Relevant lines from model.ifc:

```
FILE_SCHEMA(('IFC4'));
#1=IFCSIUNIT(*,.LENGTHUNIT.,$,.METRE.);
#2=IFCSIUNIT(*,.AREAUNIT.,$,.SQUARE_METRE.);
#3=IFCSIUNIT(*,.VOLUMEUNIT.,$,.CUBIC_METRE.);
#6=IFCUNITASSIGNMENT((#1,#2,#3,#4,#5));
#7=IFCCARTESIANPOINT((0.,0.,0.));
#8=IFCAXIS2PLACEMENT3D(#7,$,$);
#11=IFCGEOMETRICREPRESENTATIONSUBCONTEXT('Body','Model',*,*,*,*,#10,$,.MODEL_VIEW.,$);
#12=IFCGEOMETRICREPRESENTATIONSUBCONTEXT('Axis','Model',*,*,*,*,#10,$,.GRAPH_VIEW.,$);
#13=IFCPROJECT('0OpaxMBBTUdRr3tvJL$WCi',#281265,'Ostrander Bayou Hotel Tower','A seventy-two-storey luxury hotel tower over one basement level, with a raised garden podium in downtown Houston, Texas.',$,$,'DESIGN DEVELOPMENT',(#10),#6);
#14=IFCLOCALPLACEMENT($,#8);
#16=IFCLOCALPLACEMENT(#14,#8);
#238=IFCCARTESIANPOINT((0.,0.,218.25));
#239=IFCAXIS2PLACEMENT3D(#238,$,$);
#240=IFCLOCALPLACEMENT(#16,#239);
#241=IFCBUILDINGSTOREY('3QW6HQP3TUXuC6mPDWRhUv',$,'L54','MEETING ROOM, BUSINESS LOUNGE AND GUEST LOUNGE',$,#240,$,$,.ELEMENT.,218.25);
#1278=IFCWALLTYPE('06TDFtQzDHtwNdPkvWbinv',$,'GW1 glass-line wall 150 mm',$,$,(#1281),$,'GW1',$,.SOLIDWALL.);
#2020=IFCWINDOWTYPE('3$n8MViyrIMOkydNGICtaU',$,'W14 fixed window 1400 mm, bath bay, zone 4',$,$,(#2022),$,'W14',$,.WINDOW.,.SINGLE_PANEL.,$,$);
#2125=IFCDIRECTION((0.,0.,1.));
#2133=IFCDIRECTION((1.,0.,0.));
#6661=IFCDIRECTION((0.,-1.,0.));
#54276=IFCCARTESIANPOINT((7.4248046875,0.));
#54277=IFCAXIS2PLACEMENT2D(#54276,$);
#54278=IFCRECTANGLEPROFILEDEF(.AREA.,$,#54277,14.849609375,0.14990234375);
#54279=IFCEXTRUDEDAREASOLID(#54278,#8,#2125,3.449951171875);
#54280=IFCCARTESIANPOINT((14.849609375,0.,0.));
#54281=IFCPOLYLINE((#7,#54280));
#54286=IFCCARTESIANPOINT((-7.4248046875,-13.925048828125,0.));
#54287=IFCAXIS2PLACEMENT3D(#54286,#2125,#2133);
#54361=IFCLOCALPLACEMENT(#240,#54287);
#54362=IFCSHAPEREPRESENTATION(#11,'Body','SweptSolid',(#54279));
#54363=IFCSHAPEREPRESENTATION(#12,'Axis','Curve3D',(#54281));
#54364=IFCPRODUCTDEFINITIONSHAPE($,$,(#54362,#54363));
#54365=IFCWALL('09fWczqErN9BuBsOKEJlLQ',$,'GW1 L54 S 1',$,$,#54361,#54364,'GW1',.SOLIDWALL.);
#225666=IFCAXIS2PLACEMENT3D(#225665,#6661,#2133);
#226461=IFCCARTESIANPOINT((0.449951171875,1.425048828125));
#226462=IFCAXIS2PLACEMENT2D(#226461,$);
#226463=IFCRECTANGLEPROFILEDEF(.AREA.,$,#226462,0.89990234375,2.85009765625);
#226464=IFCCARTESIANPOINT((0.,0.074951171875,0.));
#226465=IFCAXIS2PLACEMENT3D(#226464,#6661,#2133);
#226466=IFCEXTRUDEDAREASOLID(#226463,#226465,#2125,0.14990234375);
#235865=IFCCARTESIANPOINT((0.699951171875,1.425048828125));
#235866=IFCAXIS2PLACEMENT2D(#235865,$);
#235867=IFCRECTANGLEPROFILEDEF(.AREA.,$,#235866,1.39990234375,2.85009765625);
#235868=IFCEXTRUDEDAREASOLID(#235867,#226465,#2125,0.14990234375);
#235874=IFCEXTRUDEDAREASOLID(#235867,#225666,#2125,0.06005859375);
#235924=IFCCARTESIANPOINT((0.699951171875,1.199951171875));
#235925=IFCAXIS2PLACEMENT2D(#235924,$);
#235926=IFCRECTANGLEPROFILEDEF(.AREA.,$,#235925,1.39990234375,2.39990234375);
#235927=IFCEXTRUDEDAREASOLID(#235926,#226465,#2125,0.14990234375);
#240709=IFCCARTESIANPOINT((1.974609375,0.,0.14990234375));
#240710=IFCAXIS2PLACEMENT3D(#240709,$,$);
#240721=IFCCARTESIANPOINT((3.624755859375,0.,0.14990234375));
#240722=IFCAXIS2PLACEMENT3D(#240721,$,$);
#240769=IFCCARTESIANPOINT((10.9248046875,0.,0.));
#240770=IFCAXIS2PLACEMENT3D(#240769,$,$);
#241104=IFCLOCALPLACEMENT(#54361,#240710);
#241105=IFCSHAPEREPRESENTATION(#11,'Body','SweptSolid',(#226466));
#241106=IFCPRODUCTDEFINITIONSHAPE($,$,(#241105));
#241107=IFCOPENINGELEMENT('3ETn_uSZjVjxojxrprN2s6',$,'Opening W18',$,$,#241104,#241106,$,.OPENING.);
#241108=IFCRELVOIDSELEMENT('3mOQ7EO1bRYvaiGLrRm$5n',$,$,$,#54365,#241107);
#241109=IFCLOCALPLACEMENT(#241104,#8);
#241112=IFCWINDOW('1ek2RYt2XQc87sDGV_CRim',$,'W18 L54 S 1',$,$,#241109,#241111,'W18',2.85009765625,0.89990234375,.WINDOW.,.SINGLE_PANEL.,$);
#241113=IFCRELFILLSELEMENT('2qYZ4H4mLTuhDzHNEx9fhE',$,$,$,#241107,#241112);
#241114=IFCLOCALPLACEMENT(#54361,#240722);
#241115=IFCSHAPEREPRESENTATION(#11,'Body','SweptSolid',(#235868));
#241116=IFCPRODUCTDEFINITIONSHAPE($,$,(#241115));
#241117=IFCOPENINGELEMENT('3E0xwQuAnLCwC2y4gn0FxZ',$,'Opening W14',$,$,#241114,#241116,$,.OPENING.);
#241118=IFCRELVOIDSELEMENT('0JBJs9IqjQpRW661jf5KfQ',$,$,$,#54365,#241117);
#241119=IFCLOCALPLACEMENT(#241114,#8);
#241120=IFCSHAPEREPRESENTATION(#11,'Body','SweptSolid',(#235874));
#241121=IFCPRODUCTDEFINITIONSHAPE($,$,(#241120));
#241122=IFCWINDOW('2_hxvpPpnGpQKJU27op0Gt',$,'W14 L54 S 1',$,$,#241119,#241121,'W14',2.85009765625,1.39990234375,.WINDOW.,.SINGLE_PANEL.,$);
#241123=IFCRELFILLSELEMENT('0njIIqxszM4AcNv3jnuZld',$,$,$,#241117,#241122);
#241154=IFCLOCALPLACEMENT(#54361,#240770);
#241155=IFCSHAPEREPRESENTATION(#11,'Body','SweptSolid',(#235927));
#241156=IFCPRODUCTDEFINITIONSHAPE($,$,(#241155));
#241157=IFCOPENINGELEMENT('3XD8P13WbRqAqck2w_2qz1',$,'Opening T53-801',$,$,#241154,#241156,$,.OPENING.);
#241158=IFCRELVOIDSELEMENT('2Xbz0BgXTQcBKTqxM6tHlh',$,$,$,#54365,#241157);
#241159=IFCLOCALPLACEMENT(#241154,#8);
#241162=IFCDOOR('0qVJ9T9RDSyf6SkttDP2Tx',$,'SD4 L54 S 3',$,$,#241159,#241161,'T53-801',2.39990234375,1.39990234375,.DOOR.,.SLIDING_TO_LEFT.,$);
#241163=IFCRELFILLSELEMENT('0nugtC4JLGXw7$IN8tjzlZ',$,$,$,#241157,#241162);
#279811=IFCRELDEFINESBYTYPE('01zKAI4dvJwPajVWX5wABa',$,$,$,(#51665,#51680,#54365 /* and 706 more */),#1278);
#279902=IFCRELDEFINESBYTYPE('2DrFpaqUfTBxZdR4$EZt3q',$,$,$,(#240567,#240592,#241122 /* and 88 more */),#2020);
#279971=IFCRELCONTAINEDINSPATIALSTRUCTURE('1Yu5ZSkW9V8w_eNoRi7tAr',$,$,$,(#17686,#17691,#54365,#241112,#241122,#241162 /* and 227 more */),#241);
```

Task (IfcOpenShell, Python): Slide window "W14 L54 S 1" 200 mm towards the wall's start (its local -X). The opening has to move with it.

```python
import ifcopenshell
import ifcopenshell.api.geometry
import ifcopenshell.util.placement

model = ifcopenshell.open("model.ifc")

window = model.by_guid("2_hxvpPpnGpQKJU27op0Gt")
opening = window.FillsVoids[0].RelatingOpeningElement
wall = opening.VoidsElements[0].RelatingBuildingElement

wall_matrix = ifcopenshell.util.placement.get_local_placement(wall.ObjectPlacement)
shift = wall_matrix[:3, 0] * -0.2
before = ifcopenshell.util.placement.get_local_placement(window.ObjectPlacement)[:3, 3].copy()

# The window is placed relative to its opening, so it follows when the opening moves.
matrix = ifcopenshell.util.placement.get_local_placement(opening.ObjectPlacement)
matrix[:3, 3] += shift
ifcopenshell.api.geometry.edit_object_placement(
    model, product=opening, matrix=matrix, is_si=False, should_transform_children=True
)

after = ifcopenshell.util.placement.get_local_placement(window.ObjectPlacement)[:3, 3]
print("window moved by", (after - before).round(3) + 0.0)

model.write("model_rev.ifc")
```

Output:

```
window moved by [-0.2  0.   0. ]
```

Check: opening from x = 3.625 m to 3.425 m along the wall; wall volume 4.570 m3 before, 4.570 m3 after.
